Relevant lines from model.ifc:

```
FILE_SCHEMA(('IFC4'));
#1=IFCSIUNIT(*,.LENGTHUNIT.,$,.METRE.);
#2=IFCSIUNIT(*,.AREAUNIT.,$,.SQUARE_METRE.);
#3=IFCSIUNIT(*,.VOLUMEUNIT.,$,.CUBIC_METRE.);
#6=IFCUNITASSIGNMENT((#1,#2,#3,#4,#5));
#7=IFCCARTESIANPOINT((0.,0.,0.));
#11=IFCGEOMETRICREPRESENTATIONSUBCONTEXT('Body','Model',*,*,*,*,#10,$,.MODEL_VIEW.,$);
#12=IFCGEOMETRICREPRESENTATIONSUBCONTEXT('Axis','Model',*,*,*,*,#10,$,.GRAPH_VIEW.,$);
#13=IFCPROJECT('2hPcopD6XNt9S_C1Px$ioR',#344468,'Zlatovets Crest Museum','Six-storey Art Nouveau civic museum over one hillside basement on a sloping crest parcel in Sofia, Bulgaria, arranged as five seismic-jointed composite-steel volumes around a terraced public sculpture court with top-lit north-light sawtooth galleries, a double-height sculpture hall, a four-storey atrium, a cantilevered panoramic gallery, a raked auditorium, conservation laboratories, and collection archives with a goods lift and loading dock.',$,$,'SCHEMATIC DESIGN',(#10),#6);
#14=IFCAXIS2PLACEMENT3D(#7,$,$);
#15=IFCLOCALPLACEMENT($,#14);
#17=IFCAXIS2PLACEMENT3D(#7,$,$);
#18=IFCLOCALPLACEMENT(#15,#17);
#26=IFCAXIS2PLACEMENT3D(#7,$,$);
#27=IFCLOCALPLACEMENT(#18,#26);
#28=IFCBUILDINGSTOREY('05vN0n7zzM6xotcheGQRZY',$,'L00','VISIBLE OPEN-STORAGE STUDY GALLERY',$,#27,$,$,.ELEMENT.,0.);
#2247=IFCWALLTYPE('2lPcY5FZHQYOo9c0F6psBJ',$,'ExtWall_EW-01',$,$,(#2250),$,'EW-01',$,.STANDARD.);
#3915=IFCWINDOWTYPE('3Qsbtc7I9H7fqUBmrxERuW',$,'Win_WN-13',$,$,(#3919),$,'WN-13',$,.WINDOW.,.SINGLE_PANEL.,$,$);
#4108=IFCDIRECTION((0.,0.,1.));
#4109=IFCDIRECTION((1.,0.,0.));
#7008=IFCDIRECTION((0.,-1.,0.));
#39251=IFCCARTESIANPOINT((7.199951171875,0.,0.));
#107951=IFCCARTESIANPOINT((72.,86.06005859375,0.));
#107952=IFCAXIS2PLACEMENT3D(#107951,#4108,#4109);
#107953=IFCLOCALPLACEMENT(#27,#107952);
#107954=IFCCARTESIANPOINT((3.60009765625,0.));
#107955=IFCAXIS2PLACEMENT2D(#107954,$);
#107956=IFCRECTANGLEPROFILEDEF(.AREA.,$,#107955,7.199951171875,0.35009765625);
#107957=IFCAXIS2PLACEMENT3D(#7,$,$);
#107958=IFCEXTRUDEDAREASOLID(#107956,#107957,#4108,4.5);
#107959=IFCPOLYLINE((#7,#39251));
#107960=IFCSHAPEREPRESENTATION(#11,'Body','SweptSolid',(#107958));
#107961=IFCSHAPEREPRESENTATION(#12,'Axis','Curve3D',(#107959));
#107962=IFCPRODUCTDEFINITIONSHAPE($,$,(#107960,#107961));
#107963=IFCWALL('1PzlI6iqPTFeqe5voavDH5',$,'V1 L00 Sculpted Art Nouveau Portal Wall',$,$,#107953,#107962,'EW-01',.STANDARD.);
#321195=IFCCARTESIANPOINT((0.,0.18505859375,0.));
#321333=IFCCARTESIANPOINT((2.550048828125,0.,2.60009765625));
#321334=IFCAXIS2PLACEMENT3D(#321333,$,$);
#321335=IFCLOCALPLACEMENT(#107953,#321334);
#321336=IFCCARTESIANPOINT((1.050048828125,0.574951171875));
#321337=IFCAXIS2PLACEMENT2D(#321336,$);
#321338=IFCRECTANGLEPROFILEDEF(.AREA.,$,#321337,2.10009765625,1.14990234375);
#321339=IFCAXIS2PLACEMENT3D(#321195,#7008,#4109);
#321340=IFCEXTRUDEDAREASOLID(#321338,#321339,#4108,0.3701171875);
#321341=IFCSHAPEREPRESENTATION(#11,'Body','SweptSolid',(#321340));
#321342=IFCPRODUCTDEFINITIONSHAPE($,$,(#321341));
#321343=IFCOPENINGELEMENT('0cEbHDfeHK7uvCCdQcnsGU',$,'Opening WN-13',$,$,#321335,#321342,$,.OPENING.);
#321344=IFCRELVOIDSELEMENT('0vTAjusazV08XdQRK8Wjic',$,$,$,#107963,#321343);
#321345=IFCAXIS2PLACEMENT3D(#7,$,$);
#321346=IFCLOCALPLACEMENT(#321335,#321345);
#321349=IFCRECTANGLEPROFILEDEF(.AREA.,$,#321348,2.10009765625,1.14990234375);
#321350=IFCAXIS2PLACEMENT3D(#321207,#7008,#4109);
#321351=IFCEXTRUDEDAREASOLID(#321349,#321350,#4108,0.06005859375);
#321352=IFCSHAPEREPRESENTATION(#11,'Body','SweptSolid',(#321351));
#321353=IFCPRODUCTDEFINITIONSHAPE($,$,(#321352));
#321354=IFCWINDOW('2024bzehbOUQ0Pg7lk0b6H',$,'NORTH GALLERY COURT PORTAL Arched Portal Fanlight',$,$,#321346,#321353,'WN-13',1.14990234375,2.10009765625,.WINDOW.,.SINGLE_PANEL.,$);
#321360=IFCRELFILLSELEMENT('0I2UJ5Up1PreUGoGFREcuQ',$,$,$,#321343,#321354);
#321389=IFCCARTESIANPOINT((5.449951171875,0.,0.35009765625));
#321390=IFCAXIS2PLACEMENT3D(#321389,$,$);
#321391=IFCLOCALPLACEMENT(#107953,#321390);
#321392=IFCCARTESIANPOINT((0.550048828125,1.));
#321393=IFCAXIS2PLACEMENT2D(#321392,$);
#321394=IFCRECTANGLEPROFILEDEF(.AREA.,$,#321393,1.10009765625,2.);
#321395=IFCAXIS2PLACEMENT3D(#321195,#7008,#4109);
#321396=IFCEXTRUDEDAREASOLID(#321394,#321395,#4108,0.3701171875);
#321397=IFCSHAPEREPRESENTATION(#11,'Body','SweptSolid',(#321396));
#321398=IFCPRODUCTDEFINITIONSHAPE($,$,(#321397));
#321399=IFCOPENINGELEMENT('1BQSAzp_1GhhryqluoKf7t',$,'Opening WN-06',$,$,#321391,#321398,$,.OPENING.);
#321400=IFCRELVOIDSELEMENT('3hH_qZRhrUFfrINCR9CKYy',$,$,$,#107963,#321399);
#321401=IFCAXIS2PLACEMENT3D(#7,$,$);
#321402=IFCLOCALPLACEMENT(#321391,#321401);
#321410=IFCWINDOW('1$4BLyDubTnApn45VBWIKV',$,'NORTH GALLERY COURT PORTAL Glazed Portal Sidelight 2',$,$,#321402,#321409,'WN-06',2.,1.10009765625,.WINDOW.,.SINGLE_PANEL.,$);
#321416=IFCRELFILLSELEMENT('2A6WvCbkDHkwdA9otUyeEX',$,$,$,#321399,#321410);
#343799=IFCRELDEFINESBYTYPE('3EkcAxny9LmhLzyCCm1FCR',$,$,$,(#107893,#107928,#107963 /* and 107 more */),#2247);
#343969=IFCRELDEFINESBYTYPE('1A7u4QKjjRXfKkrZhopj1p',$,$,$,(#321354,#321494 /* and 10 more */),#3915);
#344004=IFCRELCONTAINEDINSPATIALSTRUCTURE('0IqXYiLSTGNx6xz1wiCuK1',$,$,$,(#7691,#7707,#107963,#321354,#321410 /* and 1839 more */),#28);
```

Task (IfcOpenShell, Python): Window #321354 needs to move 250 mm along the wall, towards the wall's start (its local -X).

```python
import ifcopenshell
import ifcopenshell.api.geometry
import ifcopenshell.util.placement

model = ifcopenshell.open("model.ifc")

window = model.by_guid("2024bzehbOUQ0Pg7lk0b6H")
opening = window.FillsVoids[0].RelatingOpeningElement
wall = opening.VoidsElements[0].RelatingBuildingElement

wall_matrix = ifcopenshell.util.placement.get_local_placement(wall.ObjectPlacement)
shift = wall_matrix[:3, 0] * -0.25
before = ifcopenshell.util.placement.get_local_placement(window.ObjectPlacement)[:3, 3].copy()

# The window is placed relative to its opening, so it follows when the opening moves.
matrix = ifcopenshell.util.placement.get_local_placement(opening.ObjectPlacement)
matrix[:3, 3] += shift
ifcopenshell.api.geometry.edit_object_placement(
    model, product=opening, matrix=matrix, is_si=False, should_transform_children=True
)

after = ifcopenshell.util.placement.get_local_placement(window.ObjectPlacement)[:3, 3]
print("window moved by", (after - before).round(3) + 0.0)

model.write("model_updated.ifc")
```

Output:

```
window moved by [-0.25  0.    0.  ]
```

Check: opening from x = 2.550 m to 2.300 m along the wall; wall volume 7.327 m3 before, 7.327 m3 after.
